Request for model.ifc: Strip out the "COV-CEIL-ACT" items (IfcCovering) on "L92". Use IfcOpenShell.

First a look at what the model holds.

```python
import ifcopenshell
import ifcopenshell.util.element

model = ifcopenshell.open("model.ifc")
print(model.schema)
storey = next(s for s in model.by_type("IfcBuildingStorey") if s.Name == "L92")
coverings = [e for e in ifcopenshell.util.element.get_decomposition(storey) if e.is_a("IfcCovering")]
seen = {}
for e in coverings:
    element_type = ifcopenshell.util.element.get_type(e)
    name = element_type.Name if element_type not in (None, e) else None
    seen[name] = seen.get(name, 0) + 1
for name, count in sorted(seen.items(), key=str):
    print(count, "x", name)
```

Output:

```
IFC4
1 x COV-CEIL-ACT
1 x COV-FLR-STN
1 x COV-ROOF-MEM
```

```python
import ifcopenshell
import ifcopenshell.api.root
import ifcopenshell.util.element

model = ifcopenshell.open("model.ifc")

storey = next(s for s in model.by_type("IfcBuildingStorey") if s.Name == "L92")
coverings = [e for e in ifcopenshell.util.element.get_decomposition(storey) if e.is_a("IfcCovering")]
targets = [e for e in coverings if (t := ifcopenshell.util.element.get_type(e)) not in (None, e) and t.Name == "COV-CEIL-ACT"]

for e in targets:
    ifcopenshell.api.root.remove_product(model, product=e)
print(len(targets), "removed")

model.write("model_v2.ifc")
```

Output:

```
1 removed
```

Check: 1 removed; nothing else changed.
